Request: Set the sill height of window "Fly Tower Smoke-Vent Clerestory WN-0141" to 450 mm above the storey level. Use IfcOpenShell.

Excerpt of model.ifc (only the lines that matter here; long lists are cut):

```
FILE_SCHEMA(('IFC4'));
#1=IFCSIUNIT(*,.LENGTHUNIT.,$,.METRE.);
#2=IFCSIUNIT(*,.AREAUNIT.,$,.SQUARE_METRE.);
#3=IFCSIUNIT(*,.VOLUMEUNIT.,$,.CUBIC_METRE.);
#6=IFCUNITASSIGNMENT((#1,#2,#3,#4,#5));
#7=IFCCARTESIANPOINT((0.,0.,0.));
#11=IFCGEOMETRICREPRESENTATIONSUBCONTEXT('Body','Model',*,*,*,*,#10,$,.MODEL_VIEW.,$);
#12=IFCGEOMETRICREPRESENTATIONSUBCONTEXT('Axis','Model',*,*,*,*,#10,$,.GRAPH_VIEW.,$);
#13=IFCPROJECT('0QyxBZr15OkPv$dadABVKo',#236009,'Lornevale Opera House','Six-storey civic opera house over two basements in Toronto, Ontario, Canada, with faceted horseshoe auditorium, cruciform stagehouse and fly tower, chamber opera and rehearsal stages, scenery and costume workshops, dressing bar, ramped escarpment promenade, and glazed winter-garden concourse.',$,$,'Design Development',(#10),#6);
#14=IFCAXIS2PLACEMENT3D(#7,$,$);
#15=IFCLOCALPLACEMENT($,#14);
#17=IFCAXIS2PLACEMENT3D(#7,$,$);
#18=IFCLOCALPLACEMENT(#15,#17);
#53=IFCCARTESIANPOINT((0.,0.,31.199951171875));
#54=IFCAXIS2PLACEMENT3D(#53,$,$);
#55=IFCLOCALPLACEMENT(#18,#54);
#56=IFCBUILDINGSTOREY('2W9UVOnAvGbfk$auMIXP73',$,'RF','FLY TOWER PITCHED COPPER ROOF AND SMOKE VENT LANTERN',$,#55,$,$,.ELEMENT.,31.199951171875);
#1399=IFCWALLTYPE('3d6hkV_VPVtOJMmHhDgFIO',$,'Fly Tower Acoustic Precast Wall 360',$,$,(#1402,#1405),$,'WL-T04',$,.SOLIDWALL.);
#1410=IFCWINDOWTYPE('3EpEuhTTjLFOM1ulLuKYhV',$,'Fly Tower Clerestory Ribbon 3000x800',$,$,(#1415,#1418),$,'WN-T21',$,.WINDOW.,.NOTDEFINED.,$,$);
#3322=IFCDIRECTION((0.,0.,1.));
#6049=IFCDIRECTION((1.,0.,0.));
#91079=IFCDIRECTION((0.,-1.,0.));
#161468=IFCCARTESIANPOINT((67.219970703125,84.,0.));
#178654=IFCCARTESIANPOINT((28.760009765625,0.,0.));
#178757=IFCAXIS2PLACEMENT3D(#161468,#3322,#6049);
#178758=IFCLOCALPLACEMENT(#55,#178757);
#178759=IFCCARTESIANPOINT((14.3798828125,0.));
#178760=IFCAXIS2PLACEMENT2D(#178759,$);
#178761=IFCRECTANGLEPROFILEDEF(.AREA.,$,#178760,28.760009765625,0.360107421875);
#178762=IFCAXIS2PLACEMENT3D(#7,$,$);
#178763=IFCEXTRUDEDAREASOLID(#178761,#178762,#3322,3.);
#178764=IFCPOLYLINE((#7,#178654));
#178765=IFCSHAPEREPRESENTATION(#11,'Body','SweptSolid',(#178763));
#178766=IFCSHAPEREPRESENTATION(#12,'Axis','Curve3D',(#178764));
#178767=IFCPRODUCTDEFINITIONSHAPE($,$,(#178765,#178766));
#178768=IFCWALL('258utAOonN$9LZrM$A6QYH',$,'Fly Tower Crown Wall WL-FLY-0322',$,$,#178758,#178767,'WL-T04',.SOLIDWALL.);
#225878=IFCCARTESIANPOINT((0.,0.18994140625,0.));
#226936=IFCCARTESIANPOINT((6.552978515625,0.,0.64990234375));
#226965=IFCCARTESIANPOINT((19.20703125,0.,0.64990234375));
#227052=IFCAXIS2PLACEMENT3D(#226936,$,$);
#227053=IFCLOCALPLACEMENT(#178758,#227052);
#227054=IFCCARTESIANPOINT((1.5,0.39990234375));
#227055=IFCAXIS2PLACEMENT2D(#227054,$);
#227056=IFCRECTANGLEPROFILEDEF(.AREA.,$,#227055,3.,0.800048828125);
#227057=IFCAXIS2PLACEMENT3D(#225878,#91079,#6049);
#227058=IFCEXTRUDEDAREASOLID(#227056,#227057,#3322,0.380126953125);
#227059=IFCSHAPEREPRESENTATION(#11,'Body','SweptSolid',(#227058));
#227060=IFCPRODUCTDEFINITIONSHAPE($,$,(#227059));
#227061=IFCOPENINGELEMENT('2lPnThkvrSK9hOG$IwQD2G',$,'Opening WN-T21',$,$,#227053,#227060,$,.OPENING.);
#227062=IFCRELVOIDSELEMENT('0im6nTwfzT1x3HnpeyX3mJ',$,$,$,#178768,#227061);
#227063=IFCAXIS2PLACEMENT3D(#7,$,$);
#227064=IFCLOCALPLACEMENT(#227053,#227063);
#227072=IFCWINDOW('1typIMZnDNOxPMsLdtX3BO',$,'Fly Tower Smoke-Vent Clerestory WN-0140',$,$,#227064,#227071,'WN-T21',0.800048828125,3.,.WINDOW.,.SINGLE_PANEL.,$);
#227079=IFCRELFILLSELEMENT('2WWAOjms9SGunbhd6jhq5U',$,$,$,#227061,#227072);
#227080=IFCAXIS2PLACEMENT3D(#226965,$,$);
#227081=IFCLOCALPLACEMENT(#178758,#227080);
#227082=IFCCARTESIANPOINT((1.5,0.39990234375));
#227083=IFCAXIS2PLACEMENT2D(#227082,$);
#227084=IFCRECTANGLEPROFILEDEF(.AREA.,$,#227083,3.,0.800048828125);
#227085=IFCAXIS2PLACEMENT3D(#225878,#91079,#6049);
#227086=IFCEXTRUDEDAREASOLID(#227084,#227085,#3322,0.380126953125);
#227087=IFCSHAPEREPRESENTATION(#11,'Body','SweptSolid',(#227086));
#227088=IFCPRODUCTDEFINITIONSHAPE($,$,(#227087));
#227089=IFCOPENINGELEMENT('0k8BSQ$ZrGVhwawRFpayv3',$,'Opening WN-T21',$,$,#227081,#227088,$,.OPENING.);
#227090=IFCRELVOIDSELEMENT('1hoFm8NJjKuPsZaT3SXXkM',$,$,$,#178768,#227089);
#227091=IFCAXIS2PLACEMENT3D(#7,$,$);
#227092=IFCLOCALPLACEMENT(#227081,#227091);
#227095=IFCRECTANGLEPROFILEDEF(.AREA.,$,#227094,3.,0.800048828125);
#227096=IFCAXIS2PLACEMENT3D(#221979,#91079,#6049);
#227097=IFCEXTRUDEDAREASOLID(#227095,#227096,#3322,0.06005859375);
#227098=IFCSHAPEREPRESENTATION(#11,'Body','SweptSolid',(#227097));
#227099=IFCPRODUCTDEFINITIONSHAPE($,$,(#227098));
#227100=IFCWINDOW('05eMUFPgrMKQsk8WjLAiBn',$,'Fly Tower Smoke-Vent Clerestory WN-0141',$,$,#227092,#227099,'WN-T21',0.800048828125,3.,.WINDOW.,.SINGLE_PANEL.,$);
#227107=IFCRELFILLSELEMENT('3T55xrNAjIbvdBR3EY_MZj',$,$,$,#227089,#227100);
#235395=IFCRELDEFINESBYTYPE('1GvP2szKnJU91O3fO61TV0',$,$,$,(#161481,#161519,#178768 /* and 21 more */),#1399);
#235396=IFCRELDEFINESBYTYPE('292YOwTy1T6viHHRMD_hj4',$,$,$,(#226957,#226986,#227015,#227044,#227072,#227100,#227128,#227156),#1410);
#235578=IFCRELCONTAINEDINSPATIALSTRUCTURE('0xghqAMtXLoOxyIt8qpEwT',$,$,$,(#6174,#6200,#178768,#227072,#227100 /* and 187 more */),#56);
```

```python
import numpy as np
import ifcopenshell
import ifcopenshell.api.geometry
import ifcopenshell.geom
import ifcopenshell.util.element
import ifcopenshell.util.placement
import ifcopenshell.util.shape
import ifcopenshell.util.unit

model = ifcopenshell.open("model.ifc")
unit_scale = ifcopenshell.util.unit.calculate_unit_scale(model)

window = model.by_id(227100)
opening = window.FillsVoids[0].RelatingOpeningElement
storey = ifcopenshell.util.element.get_container(window, ifc_class="IfcBuildingStorey")
level = ifcopenshell.util.placement.get_local_placement(storey.ObjectPlacement)[2, 3]

# The opening's origin need not be at the sill, so measure its lowest point.
shape = ifcopenshell.geom.create_shape(ifcopenshell.geom.settings(), opening)
bottom = ifcopenshell.util.shape.get_shape_bottom_elevation(shape, shape.geometry) / unit_scale
dz = level + 0.45 / unit_scale - bottom

shift = np.array([0.0, 0.0, dz])
# The window is placed relative to its opening, so it follows when the opening moves.
matrix = ifcopenshell.util.placement.get_local_placement(opening.ObjectPlacement)
matrix[:3, 3] += shift
ifcopenshell.api.geometry.edit_object_placement(
    model, product=opening, matrix=matrix, is_si=False, should_transform_children=True
)

print(f"moved by {dz * unit_scale:+.3f} m")

model.write("model_v2.ifc")
```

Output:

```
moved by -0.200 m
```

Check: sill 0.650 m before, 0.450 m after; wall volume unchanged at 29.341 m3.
